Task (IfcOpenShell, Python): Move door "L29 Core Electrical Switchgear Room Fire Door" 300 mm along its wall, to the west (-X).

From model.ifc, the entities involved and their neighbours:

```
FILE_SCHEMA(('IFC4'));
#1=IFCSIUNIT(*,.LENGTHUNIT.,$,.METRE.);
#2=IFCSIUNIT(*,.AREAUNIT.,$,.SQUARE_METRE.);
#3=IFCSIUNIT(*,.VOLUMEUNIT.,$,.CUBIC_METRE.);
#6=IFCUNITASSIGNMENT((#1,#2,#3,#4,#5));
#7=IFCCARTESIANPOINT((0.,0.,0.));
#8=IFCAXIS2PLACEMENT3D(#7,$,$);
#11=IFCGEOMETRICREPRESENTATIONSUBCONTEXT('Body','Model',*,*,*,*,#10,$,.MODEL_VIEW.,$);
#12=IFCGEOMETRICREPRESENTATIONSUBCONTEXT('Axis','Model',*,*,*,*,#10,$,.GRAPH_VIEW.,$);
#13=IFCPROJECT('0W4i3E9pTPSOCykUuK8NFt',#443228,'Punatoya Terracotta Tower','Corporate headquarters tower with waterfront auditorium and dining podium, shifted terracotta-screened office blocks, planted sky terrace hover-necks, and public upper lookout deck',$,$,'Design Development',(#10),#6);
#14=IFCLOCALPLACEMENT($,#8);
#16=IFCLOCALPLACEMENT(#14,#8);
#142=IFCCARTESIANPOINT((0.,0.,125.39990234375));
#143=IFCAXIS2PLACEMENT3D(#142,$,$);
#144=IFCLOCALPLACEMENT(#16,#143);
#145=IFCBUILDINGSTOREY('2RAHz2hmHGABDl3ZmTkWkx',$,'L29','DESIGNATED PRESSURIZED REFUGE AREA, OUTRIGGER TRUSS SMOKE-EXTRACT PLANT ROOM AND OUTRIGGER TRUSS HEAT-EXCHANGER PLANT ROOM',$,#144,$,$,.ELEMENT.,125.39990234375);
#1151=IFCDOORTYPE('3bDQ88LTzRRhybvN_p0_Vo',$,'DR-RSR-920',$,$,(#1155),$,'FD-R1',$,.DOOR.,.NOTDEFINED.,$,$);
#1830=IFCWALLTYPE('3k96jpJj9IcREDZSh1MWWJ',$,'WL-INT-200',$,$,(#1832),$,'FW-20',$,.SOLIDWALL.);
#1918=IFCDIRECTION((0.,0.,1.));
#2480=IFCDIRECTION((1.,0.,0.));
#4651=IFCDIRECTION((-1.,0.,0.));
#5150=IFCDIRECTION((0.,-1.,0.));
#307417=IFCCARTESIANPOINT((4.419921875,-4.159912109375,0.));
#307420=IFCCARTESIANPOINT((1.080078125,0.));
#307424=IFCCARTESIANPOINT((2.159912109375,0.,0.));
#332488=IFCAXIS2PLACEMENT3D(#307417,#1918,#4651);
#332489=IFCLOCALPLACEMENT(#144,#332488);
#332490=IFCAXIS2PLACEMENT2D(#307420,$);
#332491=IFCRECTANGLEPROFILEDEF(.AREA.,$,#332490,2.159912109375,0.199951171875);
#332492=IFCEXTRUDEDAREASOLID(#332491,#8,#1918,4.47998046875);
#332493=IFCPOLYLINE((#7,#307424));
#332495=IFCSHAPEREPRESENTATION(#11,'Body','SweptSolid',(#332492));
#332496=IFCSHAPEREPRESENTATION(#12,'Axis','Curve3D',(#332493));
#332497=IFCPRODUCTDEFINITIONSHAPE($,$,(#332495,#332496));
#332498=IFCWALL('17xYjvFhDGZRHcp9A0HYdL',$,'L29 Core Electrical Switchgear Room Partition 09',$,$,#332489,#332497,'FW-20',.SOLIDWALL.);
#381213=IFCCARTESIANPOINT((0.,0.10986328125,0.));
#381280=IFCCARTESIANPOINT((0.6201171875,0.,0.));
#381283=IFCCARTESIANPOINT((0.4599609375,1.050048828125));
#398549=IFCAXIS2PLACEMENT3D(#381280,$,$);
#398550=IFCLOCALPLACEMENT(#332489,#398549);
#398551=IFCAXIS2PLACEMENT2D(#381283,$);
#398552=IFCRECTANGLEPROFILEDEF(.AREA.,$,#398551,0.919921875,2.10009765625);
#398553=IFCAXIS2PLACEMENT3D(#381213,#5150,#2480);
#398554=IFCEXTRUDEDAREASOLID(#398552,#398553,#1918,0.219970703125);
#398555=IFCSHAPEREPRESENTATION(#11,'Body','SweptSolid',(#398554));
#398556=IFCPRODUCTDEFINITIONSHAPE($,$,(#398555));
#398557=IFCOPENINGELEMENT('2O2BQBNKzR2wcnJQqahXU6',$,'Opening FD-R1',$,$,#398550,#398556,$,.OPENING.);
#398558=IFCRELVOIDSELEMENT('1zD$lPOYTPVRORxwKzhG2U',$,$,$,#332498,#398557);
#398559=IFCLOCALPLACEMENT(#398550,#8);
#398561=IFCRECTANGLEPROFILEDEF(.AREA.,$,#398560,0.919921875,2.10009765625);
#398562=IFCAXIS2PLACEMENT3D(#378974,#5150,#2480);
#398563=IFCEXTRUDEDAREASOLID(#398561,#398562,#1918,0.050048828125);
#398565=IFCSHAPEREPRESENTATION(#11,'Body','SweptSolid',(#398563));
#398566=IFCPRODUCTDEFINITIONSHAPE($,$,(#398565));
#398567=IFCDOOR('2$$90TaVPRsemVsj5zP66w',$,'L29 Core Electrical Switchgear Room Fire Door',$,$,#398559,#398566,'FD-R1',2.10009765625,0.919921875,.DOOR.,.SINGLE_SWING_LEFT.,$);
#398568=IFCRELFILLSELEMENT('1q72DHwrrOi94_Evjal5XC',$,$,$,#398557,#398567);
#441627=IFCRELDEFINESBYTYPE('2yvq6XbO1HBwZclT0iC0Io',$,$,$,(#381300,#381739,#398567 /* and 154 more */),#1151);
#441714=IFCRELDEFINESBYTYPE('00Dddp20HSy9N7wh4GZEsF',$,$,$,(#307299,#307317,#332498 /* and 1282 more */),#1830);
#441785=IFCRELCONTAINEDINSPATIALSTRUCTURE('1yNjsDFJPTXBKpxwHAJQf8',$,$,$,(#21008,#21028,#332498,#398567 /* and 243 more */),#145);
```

```python
import ifcopenshell
import ifcopenshell.api.geometry
import ifcopenshell.util.placement

model = ifcopenshell.open("model.ifc")

door = model.by_guid("2$$90TaVPRsemVsj5zP66w")
opening = door.FillsVoids[0].RelatingOpeningElement
wall = opening.VoidsElements[0].RelatingBuildingElement

wall_matrix = ifcopenshell.util.placement.get_local_placement(wall.ObjectPlacement)
shift = wall_matrix[:3, 0] * 0.3
before = ifcopenshell.util.placement.get_local_placement(door.ObjectPlacement)[:3, 3].copy()

# The door is placed relative to its opening, so it follows when the opening moves.
matrix = ifcopenshell.util.placement.get_local_placement(opening.ObjectPlacement)
matrix[:3, 3] += shift
ifcopenshell.api.geometry.edit_object_placement(
    model, product=opening, matrix=matrix, is_si=False, should_transform_children=True
)

after = ifcopenshell.util.placement.get_local_placement(door.ObjectPlacement)[:3, 3]
print("door moved by", (after - before).round(3) + 0.0)

model.write("model_v2.ifc")
```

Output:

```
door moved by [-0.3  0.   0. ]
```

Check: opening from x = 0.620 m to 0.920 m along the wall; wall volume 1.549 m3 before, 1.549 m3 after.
